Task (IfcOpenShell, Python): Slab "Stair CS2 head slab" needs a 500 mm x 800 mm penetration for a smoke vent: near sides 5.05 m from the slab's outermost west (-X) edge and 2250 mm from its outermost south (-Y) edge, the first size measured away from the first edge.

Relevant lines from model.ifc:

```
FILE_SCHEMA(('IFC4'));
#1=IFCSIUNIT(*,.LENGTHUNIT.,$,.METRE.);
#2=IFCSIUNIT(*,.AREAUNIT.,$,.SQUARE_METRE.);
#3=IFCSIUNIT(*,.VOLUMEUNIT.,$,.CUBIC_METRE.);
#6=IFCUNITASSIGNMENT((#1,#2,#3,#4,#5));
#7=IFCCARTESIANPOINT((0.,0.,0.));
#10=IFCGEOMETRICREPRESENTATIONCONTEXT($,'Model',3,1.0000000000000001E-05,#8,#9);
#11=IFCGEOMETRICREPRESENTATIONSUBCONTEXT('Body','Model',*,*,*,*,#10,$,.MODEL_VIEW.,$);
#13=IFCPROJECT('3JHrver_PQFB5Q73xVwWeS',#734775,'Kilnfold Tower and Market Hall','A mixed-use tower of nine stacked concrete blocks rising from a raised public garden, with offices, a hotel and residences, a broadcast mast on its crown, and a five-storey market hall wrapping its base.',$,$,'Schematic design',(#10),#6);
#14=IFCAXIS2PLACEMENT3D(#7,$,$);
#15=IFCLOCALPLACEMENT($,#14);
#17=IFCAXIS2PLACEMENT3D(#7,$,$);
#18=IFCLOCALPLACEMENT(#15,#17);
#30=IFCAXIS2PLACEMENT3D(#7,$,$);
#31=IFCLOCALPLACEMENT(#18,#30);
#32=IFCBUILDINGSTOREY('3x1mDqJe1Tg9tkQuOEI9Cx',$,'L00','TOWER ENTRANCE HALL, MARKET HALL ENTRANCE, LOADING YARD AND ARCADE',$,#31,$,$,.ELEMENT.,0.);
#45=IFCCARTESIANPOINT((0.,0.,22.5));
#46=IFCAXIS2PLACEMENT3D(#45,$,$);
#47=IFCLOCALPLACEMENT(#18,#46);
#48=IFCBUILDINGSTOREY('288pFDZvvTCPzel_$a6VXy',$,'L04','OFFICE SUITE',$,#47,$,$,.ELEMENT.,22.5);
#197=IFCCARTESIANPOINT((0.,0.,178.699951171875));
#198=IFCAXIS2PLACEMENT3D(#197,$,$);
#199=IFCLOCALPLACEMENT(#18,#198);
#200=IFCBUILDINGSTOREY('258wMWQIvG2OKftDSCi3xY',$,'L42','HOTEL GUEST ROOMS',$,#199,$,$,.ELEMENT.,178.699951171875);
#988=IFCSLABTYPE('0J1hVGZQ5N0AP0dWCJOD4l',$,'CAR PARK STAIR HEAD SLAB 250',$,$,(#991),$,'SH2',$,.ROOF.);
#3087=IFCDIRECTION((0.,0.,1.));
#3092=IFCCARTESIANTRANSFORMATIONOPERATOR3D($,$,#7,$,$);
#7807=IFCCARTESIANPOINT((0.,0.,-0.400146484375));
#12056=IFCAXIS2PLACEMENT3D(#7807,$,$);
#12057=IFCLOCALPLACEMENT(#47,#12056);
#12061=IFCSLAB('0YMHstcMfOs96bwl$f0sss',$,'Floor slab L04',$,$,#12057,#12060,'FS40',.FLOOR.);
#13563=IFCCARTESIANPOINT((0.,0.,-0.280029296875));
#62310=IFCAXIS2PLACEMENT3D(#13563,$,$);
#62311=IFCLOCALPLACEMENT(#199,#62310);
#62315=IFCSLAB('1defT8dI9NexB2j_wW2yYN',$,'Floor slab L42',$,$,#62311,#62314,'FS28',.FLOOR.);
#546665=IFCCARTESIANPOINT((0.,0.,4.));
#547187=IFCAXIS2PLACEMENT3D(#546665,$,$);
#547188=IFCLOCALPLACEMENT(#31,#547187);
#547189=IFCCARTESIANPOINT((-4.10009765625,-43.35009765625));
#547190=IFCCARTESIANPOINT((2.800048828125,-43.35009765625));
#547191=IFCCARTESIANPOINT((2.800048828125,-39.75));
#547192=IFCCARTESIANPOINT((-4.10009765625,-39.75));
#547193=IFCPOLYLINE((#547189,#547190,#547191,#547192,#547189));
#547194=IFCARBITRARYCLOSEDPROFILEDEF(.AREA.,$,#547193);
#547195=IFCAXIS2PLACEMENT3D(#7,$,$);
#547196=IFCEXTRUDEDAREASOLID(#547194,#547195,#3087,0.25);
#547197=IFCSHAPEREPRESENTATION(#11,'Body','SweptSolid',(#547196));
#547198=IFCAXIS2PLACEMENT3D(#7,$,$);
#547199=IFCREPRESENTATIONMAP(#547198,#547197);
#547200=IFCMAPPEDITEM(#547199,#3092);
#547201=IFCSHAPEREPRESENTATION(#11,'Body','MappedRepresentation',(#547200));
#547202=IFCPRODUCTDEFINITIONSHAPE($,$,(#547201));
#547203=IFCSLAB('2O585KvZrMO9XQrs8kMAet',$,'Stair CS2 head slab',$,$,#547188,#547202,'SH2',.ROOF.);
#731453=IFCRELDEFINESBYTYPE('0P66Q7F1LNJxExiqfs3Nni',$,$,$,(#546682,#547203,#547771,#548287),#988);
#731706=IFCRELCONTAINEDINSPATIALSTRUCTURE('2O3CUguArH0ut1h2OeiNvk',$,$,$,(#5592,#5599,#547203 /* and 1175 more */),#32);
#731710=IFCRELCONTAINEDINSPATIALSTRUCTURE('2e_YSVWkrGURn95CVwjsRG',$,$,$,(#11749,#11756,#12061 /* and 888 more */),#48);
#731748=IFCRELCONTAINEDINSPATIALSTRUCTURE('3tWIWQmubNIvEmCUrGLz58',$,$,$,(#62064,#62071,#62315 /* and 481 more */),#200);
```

```python
import numpy as np
import ifcopenshell
import ifcopenshell.api.feature
import ifcopenshell.api.geometry
import ifcopenshell.api.root
import ifcopenshell.geom
import ifcopenshell.util.placement
import ifcopenshell.util.representation
import ifcopenshell.util.shape
import ifcopenshell.util.unit

model = ifcopenshell.open("model.ifc")
unit_scale = ifcopenshell.util.unit.calculate_unit_scale(model)
settings = ifcopenshell.geom.settings()


def volume(element):
    """Net volume in cubic metres, openings subtracted."""
    shape = ifcopenshell.geom.create_shape(settings, element)
    return ifcopenshell.util.shape.get_volume(shape.geometry)


slab = model.by_guid("2O585KvZrMO9XQrs8kMAet")
before = volume(slab)

# Extent in the slab's own axes, in metres. The edges named are its -X and -Y sides.
slab_shape = ifcopenshell.geom.create_shape(settings, slab)
vertices = ifcopenshell.util.shape.get_vertices(slab_shape.geometry)
x_min, y_min, bottom = vertices.min(axis=0)
top = vertices[:, 2].max()

opening = ifcopenshell.api.root.create_entity(model, ifc_class="IfcOpeningElement", name="Smoke vent opening", predefined_type="OPENING")
context = ifcopenshell.util.representation.get_context(model, "Model", "Body", "MODEL_VIEW")
width, depth = 0.5, 0.8
outline = [(0.0, 0.0), (width, 0.0), (width, depth), (0.0, depth), (0.0, 0.0)]
# Overshoot both faces by 50 mm so the cut is clean.
shape = ifcopenshell.api.geometry.add_slab_representation(
    model, context=context, depth=top - bottom + 0.1, polyline=outline
)
ifcopenshell.api.geometry.assign_representation(model, product=opening, representation=shape)

matrix = ifcopenshell.util.placement.get_local_placement(slab.ObjectPlacement)
matrix[:, 3] = matrix @ np.append(np.array([x_min + 5.05, y_min + 2.25, bottom - 0.05]) / unit_scale, 1.0)
ifcopenshell.api.geometry.edit_object_placement(model, product=opening, matrix=matrix, is_si=False)
ifcopenshell.api.feature.add_feature(model, feature=opening, element=slab)

after = volume(slab)

print(f"slab volume {before:.3f} -> {after:.3f} m3")

model.write("model_rev.ifc")
```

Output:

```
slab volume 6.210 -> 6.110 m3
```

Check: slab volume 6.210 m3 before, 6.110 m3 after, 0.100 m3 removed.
